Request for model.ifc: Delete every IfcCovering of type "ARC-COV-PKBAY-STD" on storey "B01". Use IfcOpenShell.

First a look at what the model holds.

```python
import ifcopenshell
import ifcopenshell.util.element

model = ifcopenshell.open("model.ifc")
print(model.schema)
storey = next(s for s in model.by_type("IfcBuildingStorey") if s.Name == "B01")
coverings = [e for e in ifcopenshell.util.element.get_decomposition(storey) if e.is_a("IfcCovering")]
seen = {}
for e in coverings:
    element_type = ifcopenshell.util.element.get_type(e)
    name = element_type.Name if element_type not in (None, e) else None
    seen[name] = seen.get(name, 0) + 1
for name, count in sorted(seen.items(), key=str):
    print(count, "x", name)
```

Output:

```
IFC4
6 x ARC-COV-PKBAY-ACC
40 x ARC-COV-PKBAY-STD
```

```python
import ifcopenshell
import ifcopenshell.api.root
import ifcopenshell.util.element

model = ifcopenshell.open("model.ifc")

storey = next(s for s in model.by_type("IfcBuildingStorey") if s.Name == "B01")
coverings = [e for e in ifcopenshell.util.element.get_decomposition(storey) if e.is_a("IfcCovering")]
targets = [e for e in coverings if (t := ifcopenshell.util.element.get_type(e)) not in (None, e) and t.Name == "ARC-COV-PKBAY-STD"]

for e in targets:
    ifcopenshell.api.root.remove_product(model, product=e)
print(len(targets), "removed")

model.write("model_edited.ifc")
```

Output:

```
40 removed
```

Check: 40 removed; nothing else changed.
